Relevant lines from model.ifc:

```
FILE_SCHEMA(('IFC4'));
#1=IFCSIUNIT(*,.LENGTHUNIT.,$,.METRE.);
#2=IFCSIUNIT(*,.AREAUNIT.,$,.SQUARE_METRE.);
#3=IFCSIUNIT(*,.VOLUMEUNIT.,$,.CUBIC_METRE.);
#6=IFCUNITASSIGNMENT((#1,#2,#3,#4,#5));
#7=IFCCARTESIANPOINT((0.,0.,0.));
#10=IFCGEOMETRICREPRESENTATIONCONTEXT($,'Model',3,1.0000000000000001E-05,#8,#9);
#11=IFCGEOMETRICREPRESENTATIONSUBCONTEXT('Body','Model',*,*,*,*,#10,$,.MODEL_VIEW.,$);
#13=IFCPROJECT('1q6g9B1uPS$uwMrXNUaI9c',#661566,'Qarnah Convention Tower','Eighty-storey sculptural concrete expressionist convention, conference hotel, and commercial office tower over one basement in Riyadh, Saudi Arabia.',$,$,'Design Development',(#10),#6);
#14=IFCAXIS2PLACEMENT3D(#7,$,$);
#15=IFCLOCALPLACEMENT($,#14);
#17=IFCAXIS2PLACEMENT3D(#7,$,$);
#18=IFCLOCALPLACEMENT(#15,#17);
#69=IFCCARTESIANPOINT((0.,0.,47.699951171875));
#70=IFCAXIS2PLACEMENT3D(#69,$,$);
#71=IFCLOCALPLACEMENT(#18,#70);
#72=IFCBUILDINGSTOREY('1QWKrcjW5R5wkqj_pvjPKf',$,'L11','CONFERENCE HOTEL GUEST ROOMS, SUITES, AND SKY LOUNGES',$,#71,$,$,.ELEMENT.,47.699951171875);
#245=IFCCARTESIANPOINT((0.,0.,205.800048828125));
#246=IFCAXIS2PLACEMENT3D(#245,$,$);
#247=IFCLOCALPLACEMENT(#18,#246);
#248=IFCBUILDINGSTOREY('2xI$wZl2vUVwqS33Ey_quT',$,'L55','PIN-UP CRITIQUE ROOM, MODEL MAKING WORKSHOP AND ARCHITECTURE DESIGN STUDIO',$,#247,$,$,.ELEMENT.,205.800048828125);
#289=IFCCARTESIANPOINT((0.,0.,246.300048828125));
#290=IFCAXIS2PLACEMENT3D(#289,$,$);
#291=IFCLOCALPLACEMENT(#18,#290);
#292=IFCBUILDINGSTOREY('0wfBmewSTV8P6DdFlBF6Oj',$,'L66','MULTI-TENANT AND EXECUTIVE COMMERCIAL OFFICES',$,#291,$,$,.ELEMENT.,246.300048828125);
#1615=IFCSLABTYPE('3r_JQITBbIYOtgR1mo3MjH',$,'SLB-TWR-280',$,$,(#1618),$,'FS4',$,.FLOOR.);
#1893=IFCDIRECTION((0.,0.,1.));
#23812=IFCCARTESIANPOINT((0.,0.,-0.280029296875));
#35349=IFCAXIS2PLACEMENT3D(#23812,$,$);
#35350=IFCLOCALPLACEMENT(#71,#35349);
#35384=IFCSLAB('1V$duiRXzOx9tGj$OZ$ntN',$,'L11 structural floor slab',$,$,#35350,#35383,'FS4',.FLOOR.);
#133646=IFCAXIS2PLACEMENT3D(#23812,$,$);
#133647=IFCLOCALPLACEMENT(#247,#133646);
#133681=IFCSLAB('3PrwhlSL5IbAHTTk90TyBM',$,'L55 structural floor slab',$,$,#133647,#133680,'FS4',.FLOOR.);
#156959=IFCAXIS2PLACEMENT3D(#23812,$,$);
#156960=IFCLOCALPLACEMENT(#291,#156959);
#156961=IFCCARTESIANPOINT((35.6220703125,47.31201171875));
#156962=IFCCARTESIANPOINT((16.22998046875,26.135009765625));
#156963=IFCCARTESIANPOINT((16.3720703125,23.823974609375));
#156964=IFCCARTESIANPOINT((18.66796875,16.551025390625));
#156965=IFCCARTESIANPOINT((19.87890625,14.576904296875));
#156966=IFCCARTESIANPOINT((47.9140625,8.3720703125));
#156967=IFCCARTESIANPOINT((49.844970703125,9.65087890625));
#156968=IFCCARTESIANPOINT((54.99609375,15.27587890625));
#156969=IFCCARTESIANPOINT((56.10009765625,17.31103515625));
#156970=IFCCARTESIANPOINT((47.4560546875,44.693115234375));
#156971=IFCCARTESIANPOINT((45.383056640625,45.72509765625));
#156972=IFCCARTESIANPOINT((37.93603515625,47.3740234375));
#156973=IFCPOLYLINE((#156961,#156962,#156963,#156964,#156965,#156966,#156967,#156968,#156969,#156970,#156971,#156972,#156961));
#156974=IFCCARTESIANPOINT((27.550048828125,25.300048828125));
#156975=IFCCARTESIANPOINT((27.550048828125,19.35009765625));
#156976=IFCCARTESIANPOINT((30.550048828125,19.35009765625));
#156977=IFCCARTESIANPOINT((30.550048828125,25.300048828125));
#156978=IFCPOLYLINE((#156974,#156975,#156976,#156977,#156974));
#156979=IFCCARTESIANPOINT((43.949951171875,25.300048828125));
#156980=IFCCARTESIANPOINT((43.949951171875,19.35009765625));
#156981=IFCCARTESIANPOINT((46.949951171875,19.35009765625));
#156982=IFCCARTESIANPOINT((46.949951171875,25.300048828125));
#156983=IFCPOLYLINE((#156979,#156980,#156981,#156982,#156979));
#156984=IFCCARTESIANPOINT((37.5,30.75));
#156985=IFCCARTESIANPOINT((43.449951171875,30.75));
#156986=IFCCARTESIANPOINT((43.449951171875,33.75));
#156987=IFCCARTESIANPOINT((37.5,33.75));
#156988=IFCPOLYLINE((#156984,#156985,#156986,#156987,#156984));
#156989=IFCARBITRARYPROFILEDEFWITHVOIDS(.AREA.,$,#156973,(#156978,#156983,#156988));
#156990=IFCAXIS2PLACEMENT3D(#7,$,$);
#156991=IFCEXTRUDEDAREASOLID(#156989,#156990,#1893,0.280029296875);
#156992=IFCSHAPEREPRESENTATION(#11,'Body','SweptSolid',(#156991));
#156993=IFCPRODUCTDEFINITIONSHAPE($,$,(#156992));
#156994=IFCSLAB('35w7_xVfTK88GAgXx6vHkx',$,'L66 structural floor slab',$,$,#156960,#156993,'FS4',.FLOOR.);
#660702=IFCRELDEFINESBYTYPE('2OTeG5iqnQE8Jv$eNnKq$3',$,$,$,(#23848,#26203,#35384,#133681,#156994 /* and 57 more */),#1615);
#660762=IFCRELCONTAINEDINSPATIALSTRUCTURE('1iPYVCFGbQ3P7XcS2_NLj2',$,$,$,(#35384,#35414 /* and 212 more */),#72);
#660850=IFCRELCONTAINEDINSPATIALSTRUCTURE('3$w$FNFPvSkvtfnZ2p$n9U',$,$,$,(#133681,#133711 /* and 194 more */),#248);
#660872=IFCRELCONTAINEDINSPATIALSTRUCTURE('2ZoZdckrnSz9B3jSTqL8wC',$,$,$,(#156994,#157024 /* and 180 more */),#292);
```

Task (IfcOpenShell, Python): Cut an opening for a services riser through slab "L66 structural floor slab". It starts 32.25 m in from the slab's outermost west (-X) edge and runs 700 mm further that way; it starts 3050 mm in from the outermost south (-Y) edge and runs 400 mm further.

```python
import numpy as np
import ifcopenshell
import ifcopenshell.api.feature
import ifcopenshell.api.geometry
import ifcopenshell.api.root
import ifcopenshell.geom
import ifcopenshell.util.placement
import ifcopenshell.util.representation
import ifcopenshell.util.shape
import ifcopenshell.util.unit

model = ifcopenshell.open("model.ifc")
unit_scale = ifcopenshell.util.unit.calculate_unit_scale(model)
settings = ifcopenshell.geom.settings()


def volume(element):
    """Net volume in cubic metres, openings subtracted."""
    shape = ifcopenshell.geom.create_shape(settings, element)
    return ifcopenshell.util.shape.get_volume(shape.geometry)


slab = model.by_id(156994)
before = volume(slab)

# Extent in the slab's own axes, in metres. The edges named are its -X and -Y sides.
slab_shape = ifcopenshell.geom.create_shape(settings, slab)
vertices = ifcopenshell.util.shape.get_vertices(slab_shape.geometry)
x_min, y_min, bottom = vertices.min(axis=0)
top = vertices[:, 2].max()

opening = ifcopenshell.api.root.create_entity(model, ifc_class="IfcOpeningElement", name="Services riser opening", predefined_type="OPENING")
context = ifcopenshell.util.representation.get_context(model, "Model", "Body", "MODEL_VIEW")
width, depth = 0.7, 0.4
outline = [(0.0, 0.0), (width, 0.0), (width, depth), (0.0, depth), (0.0, 0.0)]
# Overshoot both faces by 50 mm so the cut is clean.
shape = ifcopenshell.api.geometry.add_slab_representation(
    model, context=context, depth=top - bottom + 0.1, polyline=outline
)
ifcopenshell.api.geometry.assign_representation(model, product=opening, representation=shape)

matrix = ifcopenshell.util.placement.get_local_placement(slab.ObjectPlacement)
matrix[:, 3] = matrix @ np.append(np.array([x_min + 32.25, y_min + 3.05, bottom - 0.05]) / unit_scale, 1.0)
ifcopenshell.api.geometry.edit_object_placement(model, product=opening, matrix=matrix, is_si=False)
ifcopenshell.api.feature.add_feature(model, feature=opening, element=slab)

after = volume(slab)

print(f"slab volume {before:.3f} -> {after:.3f} m3")

model.write("model_updated.ifc")
```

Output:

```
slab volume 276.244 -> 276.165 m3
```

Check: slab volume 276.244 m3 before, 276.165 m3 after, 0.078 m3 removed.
